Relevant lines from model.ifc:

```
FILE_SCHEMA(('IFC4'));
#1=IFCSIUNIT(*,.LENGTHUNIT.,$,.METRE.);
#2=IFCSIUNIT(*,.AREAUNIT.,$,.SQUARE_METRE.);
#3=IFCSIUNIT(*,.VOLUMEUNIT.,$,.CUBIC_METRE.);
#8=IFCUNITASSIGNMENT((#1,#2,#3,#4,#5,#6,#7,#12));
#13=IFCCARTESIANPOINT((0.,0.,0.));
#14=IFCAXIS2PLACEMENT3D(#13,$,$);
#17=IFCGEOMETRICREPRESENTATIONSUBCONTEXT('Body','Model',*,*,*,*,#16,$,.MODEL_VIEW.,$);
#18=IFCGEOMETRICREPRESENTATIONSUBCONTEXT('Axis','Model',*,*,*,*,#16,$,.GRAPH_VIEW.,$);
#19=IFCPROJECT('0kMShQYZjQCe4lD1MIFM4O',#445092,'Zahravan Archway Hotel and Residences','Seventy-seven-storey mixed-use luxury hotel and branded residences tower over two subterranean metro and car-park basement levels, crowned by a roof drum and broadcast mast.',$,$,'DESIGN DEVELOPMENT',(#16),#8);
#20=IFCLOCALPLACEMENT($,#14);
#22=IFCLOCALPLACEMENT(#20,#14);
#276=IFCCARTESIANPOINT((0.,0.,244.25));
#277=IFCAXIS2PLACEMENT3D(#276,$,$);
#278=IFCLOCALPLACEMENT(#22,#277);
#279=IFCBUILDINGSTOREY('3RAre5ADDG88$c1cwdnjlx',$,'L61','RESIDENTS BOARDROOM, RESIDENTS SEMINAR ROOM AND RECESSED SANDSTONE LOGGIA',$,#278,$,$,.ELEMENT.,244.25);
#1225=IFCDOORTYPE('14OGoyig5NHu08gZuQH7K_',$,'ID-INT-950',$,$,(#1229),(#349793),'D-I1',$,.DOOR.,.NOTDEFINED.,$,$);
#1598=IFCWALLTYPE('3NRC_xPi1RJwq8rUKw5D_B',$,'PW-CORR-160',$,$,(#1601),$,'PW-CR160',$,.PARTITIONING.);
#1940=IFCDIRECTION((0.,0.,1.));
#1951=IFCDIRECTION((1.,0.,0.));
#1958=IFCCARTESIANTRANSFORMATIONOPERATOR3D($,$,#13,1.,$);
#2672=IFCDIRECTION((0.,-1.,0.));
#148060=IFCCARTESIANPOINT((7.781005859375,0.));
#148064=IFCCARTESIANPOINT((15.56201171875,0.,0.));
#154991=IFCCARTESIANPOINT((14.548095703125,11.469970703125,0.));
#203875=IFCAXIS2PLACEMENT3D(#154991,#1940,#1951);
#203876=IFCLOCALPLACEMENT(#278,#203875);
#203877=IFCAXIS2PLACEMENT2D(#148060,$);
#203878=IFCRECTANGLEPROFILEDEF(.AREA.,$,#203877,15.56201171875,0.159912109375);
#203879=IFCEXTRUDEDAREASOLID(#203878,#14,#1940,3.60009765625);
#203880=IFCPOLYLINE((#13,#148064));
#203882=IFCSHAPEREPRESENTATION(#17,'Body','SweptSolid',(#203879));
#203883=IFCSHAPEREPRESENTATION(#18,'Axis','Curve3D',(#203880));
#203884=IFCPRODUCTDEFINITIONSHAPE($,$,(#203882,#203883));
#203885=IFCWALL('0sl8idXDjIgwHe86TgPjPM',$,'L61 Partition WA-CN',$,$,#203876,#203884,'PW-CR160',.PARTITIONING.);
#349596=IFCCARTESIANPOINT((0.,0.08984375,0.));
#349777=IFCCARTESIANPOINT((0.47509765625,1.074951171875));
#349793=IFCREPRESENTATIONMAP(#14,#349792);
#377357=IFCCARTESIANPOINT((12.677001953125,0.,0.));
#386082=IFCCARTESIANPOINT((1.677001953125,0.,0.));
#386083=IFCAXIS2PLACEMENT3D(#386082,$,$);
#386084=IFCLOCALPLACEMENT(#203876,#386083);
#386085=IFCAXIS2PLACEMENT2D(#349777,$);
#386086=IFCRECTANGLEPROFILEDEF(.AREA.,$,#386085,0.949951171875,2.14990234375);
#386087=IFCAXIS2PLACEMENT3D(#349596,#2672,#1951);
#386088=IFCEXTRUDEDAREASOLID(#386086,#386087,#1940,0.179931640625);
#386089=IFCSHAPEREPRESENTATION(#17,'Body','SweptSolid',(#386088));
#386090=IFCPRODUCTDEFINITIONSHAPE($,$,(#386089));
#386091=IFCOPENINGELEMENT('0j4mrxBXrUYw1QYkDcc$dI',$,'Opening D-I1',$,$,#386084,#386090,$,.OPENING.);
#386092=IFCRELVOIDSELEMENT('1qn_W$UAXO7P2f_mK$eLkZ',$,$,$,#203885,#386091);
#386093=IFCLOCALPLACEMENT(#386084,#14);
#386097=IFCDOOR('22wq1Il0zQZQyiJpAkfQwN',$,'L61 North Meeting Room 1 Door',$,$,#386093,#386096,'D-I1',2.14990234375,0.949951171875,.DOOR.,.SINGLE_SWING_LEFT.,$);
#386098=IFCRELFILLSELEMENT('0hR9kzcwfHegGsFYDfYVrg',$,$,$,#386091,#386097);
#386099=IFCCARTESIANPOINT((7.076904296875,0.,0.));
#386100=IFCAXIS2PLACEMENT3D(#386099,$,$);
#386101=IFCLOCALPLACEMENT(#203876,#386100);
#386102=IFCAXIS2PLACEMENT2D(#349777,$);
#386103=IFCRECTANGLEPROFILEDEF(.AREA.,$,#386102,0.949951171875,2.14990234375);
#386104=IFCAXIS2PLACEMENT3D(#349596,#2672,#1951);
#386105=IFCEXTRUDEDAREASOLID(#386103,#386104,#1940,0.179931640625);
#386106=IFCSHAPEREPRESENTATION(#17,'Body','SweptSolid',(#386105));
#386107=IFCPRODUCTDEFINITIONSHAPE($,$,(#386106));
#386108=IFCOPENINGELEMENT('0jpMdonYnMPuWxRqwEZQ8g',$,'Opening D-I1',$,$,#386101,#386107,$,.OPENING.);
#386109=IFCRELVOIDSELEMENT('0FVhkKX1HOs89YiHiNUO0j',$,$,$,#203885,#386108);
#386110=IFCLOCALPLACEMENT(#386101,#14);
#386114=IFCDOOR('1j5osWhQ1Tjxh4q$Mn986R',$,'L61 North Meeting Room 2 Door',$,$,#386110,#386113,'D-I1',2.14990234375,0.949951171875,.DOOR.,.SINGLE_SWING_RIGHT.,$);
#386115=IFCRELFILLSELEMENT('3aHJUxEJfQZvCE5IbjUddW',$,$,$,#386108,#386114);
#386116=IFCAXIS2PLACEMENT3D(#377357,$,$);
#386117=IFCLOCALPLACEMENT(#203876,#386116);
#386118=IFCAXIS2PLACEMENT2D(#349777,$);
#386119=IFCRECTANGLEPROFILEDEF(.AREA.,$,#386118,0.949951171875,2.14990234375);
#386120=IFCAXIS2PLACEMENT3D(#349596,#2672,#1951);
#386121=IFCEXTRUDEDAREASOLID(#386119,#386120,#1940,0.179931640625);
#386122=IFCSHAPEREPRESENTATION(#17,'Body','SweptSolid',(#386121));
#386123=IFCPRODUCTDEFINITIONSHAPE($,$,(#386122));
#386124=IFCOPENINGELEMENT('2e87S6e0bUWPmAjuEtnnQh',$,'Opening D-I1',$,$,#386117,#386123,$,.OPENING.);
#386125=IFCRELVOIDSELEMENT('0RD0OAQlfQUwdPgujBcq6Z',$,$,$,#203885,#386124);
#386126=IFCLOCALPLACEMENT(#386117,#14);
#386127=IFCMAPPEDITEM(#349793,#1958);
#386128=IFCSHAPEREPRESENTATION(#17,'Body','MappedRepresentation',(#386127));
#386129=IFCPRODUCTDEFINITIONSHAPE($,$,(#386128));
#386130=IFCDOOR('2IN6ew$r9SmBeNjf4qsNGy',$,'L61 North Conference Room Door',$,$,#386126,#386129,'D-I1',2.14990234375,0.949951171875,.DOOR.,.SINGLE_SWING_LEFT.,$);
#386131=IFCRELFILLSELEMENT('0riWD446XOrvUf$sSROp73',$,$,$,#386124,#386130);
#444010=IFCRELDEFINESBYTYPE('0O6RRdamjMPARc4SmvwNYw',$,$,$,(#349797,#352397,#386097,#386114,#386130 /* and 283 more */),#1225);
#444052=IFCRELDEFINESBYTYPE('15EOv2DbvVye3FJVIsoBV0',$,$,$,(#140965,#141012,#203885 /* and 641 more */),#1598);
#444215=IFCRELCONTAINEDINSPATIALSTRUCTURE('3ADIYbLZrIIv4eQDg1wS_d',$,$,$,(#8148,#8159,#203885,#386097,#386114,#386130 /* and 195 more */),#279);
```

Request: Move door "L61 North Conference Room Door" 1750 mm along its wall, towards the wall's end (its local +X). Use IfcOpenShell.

```python
import ifcopenshell
import ifcopenshell.api.geometry
import ifcopenshell.util.placement
import ifcopenshell.util.unit

model = ifcopenshell.open("model.ifc")
unit_scale = ifcopenshell.util.unit.calculate_unit_scale(model)

door = model.by_id(386130)
opening = door.FillsVoids[0].RelatingOpeningElement
wall = opening.VoidsElements[0].RelatingBuildingElement

wall_matrix = ifcopenshell.util.placement.get_local_placement(wall.ObjectPlacement)
shift = wall_matrix[:3, 0] * 1.75 / unit_scale
before = ifcopenshell.util.placement.get_local_placement(door.ObjectPlacement)[:3, 3].copy()

# The door is placed relative to its opening, so it follows when the opening moves.
matrix = ifcopenshell.util.placement.get_local_placement(opening.ObjectPlacement)
matrix[:3, 3] += shift
ifcopenshell.api.geometry.edit_object_placement(
    model, product=opening, matrix=matrix, is_si=False, should_transform_children=True
)

after = ifcopenshell.util.placement.get_local_placement(door.ObjectPlacement)[:3, 3]
print("door moved by", (after - before).round(3) + 0.0)

model.write("model_updated.ifc")
```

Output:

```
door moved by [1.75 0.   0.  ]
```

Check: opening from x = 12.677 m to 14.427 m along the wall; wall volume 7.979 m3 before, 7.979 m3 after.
